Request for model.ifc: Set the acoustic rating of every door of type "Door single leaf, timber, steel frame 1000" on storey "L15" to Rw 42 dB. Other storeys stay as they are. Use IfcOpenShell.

First a look at what the model holds.

```python
import ifcopenshell
import ifcopenshell.util.element

model = ifcopenshell.open("model.ifc")
print(model.schema)
storey = next(s for s in model.by_type("IfcBuildingStorey") if s.Name == "L15")
doors = [e for e in ifcopenshell.util.element.get_decomposition(storey) if e.is_a("IfcDoor")]
seen = {}
for e in doors:
    element_type = ifcopenshell.util.element.get_type(e)
    key = (element_type.Name if element_type != e and element_type else None, ifcopenshell.util.element.get_pset(e, "Pset_DoorCommon", "AcousticRating"))
    seen[key] = seen.get(key, 0) + 1
for (name, value), count in sorted(seen.items(), key=str):
    print(count, "x", name, "|", value)
```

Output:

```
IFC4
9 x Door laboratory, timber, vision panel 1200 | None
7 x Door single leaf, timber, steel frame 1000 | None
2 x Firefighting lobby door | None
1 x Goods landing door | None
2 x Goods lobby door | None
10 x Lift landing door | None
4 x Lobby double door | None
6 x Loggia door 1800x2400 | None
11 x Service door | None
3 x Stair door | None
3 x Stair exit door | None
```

```python
import ifcopenshell
import ifcopenshell.api.pset
import ifcopenshell.util.element

model = ifcopenshell.open("model.ifc")

storey = next(s for s in model.by_type("IfcBuildingStorey") if s.Name == "L15")
doors = [e for e in ifcopenshell.util.element.get_decomposition(storey) if e.is_a("IfcDoor")]

count = 0
for e in doors:
    element_type = ifcopenshell.util.element.get_type(e)
    if element_type in (None, e) or element_type.Name != "Door single leaf, timber, steel frame 1000":
        continue
    # add_pset returns the element's existing set when there is one.
    pset = ifcopenshell.api.pset.add_pset(model, product=e, name="Pset_DoorCommon")
    ifcopenshell.api.pset.edit_pset(model, pset=pset, properties={"AcousticRating": "Rw 42 dB"})
    count += 1

print(count, "doors updated")

model.write("model-out.ifc")
```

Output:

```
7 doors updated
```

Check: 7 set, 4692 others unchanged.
